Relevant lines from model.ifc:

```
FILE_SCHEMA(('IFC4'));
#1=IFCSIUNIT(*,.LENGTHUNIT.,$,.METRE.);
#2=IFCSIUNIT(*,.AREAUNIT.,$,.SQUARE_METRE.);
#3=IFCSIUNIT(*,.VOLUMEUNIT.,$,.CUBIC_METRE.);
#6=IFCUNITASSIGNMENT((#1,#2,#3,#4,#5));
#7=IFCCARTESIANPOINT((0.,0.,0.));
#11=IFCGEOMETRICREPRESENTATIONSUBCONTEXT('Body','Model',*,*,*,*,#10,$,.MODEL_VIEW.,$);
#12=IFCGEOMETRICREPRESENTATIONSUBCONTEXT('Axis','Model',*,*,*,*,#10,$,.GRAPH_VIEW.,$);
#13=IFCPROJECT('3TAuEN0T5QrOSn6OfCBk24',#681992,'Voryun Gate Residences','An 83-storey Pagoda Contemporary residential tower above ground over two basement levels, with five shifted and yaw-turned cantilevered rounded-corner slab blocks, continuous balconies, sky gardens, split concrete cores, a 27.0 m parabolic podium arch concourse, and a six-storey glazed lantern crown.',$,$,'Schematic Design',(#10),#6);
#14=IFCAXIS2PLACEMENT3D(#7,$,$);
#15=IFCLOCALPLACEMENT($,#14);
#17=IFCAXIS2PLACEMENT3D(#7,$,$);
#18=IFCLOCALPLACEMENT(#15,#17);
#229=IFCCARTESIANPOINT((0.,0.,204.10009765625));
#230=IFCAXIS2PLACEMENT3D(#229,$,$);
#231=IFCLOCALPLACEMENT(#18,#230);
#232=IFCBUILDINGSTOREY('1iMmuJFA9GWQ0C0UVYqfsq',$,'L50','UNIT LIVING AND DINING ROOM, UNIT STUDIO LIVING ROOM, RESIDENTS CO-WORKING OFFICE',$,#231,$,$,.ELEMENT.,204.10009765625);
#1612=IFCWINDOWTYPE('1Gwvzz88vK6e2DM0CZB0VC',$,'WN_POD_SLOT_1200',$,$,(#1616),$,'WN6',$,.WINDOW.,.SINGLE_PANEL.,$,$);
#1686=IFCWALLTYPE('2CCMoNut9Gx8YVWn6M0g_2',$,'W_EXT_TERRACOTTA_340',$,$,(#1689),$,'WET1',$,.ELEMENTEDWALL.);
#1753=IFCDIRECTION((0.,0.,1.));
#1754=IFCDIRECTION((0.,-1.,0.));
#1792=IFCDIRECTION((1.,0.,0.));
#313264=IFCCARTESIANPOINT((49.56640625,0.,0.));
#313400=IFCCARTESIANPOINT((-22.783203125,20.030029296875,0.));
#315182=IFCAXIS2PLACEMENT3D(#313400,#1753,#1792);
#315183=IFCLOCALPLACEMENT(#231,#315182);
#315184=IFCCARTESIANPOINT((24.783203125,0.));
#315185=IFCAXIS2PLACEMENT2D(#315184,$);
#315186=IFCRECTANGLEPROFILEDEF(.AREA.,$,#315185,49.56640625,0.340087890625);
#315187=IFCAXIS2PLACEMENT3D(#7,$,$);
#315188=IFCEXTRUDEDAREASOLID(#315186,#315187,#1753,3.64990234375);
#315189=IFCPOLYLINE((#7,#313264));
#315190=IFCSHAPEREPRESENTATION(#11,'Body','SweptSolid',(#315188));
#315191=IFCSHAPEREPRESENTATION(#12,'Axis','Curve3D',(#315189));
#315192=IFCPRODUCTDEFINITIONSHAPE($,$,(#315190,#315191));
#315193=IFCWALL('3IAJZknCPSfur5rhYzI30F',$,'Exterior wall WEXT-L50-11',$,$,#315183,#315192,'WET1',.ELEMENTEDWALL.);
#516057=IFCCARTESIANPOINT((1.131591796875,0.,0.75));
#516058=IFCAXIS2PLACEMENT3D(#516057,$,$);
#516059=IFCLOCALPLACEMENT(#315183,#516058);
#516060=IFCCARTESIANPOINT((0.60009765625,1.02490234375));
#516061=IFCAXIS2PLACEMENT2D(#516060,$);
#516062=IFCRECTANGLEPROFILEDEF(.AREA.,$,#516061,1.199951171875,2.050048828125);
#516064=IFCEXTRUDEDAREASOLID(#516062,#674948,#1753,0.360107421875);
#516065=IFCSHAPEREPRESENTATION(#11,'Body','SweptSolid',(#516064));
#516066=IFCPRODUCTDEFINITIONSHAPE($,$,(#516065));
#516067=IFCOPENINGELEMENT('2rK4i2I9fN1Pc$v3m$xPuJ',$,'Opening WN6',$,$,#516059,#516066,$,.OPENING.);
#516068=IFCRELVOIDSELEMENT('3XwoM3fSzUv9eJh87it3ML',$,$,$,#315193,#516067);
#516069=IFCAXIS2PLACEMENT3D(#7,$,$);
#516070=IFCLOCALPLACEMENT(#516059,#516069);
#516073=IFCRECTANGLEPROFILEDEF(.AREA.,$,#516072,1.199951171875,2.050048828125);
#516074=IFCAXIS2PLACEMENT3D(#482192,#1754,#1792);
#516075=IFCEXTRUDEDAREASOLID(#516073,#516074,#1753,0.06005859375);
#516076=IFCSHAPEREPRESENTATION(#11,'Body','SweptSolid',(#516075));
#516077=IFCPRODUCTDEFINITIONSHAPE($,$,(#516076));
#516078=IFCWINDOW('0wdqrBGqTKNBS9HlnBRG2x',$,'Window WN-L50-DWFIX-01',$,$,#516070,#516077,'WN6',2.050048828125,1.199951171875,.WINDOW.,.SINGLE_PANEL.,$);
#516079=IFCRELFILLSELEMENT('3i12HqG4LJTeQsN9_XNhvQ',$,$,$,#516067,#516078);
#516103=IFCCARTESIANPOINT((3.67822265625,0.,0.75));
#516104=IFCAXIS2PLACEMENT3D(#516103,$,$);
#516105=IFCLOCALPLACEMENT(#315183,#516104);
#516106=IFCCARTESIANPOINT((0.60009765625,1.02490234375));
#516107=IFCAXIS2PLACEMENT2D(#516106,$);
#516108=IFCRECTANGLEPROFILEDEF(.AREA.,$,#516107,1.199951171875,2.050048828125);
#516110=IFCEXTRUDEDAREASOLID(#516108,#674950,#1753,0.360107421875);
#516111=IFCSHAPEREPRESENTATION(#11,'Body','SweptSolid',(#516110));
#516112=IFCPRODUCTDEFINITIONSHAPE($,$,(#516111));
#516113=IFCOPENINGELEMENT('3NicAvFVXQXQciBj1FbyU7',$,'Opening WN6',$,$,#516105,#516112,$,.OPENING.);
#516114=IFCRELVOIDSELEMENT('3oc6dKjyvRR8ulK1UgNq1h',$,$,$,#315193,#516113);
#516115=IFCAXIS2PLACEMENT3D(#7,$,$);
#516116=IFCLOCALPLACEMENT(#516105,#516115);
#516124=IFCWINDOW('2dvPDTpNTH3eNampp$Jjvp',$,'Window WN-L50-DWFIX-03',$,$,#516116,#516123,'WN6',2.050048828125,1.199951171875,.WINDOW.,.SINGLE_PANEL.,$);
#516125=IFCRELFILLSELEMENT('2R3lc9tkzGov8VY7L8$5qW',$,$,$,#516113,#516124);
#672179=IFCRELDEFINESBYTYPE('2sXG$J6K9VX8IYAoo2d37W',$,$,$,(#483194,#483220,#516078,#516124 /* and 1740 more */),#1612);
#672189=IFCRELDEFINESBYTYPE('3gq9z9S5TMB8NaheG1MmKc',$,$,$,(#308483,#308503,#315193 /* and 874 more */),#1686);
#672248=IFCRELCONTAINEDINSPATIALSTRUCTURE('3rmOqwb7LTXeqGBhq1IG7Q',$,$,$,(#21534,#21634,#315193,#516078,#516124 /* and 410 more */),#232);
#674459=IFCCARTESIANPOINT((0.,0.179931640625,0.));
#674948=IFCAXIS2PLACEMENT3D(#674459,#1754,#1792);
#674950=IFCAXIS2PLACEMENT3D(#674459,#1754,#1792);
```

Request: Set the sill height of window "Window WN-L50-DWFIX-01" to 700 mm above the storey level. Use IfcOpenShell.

```python
import numpy as np
import ifcopenshell
import ifcopenshell.api.geometry
import ifcopenshell.geom
import ifcopenshell.util.element
import ifcopenshell.util.placement
import ifcopenshell.util.shape
import ifcopenshell.util.unit

model = ifcopenshell.open("model.ifc")
unit_scale = ifcopenshell.util.unit.calculate_unit_scale(model)

window = model.by_id(516078)
opening = window.FillsVoids[0].RelatingOpeningElement
storey = ifcopenshell.util.element.get_container(window, ifc_class="IfcBuildingStorey")
level = ifcopenshell.util.placement.get_local_placement(storey.ObjectPlacement)[2, 3]

# The opening's origin need not be at the sill, so measure its lowest point.
shape = ifcopenshell.geom.create_shape(ifcopenshell.geom.settings(), opening)
bottom = ifcopenshell.util.shape.get_shape_bottom_elevation(shape, shape.geometry) / unit_scale
dz = level + 0.7 / unit_scale - bottom

shift = np.array([0.0, 0.0, dz])
# The window is placed relative to its opening, so it follows when the opening moves.
matrix = ifcopenshell.util.placement.get_local_placement(opening.ObjectPlacement)
matrix[:3, 3] += shift
ifcopenshell.api.geometry.edit_object_placement(
    model, product=opening, matrix=matrix, is_si=False, should_transform_children=True
)

print(f"moved by {dz * unit_scale:+.3f} m")

model.write("model_v2.ifc")
```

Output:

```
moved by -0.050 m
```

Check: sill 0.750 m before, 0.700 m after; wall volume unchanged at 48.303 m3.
